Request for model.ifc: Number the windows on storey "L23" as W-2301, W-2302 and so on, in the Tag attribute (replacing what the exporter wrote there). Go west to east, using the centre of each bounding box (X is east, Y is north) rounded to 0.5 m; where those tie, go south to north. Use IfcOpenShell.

First a look at what the model holds.

```python
import ifcopenshell
import ifcopenshell.util.element
import ifcopenshell.util.placement

model = ifcopenshell.open("model.ifc")
print(model.schema)
storey = next(s for s in model.by_type("IfcBuildingStorey") if s.Name == "L23")
windows = [e for e in ifcopenshell.util.element.get_decomposition(storey) if e.is_a("IfcWindow")]
for e in sorted(windows, key=lambda e: e.id()):
    origin = ifcopenshell.util.placement.get_local_placement(e.ObjectPlacement)[:3, 3]
    print(e.id(), e.Tag, e.Name, origin.round(2) + 0.0, sep=" | ")
```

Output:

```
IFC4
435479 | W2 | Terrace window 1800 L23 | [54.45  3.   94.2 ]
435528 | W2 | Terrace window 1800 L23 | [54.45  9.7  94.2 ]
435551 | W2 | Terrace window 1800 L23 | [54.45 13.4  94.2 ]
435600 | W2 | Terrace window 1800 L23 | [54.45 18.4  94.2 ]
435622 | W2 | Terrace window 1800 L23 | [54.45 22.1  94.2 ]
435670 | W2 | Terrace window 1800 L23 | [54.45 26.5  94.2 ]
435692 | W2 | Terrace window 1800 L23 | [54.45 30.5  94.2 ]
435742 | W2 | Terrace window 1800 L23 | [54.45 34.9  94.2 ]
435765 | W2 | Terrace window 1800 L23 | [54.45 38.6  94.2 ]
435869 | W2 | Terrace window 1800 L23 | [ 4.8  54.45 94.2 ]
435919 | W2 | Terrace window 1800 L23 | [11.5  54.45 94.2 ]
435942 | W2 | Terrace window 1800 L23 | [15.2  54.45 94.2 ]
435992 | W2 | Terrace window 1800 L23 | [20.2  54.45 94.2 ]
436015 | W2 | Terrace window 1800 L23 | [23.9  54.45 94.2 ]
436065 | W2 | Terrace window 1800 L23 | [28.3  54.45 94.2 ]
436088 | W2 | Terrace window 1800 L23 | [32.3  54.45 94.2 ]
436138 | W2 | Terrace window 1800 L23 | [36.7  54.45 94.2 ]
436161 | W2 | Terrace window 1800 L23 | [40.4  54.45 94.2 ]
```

```python
import ifcopenshell
import ifcopenshell.geom
import ifcopenshell.util.element
import ifcopenshell.util.shape

model = ifcopenshell.open("model.ifc")
settings = ifcopenshell.geom.settings()
settings.set("use-world-coords", True)


def centre(element):
    shape = ifcopenshell.geom.create_shape(settings, element)
    return ifcopenshell.util.shape.get_bbox_centroid(shape.geometry)


storey = next(s for s in model.by_type("IfcBuildingStorey") if s.Name == "L23")
windows = [e for e in ifcopenshell.util.element.get_decomposition(storey) if e.is_a("IfcWindow")]

# Insertion points can sit at a corner or the storey origin, so sort by the geometry (in metres).
centres = {e: centre(e) for e in windows}
windows.sort(key=lambda e: (round(centres[e][0] / 0.5), centres[e][1]))

for i, e in enumerate(windows, start=1):
    number = f"W-23{i:02d}"
    e.Tag = number
    print(e.id(), number)

model.write("model_updated.ifc")
```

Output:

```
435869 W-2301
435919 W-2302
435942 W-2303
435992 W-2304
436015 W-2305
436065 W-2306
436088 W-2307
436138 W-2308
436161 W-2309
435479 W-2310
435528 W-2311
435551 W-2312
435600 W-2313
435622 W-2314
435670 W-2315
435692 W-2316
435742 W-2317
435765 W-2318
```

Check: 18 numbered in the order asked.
